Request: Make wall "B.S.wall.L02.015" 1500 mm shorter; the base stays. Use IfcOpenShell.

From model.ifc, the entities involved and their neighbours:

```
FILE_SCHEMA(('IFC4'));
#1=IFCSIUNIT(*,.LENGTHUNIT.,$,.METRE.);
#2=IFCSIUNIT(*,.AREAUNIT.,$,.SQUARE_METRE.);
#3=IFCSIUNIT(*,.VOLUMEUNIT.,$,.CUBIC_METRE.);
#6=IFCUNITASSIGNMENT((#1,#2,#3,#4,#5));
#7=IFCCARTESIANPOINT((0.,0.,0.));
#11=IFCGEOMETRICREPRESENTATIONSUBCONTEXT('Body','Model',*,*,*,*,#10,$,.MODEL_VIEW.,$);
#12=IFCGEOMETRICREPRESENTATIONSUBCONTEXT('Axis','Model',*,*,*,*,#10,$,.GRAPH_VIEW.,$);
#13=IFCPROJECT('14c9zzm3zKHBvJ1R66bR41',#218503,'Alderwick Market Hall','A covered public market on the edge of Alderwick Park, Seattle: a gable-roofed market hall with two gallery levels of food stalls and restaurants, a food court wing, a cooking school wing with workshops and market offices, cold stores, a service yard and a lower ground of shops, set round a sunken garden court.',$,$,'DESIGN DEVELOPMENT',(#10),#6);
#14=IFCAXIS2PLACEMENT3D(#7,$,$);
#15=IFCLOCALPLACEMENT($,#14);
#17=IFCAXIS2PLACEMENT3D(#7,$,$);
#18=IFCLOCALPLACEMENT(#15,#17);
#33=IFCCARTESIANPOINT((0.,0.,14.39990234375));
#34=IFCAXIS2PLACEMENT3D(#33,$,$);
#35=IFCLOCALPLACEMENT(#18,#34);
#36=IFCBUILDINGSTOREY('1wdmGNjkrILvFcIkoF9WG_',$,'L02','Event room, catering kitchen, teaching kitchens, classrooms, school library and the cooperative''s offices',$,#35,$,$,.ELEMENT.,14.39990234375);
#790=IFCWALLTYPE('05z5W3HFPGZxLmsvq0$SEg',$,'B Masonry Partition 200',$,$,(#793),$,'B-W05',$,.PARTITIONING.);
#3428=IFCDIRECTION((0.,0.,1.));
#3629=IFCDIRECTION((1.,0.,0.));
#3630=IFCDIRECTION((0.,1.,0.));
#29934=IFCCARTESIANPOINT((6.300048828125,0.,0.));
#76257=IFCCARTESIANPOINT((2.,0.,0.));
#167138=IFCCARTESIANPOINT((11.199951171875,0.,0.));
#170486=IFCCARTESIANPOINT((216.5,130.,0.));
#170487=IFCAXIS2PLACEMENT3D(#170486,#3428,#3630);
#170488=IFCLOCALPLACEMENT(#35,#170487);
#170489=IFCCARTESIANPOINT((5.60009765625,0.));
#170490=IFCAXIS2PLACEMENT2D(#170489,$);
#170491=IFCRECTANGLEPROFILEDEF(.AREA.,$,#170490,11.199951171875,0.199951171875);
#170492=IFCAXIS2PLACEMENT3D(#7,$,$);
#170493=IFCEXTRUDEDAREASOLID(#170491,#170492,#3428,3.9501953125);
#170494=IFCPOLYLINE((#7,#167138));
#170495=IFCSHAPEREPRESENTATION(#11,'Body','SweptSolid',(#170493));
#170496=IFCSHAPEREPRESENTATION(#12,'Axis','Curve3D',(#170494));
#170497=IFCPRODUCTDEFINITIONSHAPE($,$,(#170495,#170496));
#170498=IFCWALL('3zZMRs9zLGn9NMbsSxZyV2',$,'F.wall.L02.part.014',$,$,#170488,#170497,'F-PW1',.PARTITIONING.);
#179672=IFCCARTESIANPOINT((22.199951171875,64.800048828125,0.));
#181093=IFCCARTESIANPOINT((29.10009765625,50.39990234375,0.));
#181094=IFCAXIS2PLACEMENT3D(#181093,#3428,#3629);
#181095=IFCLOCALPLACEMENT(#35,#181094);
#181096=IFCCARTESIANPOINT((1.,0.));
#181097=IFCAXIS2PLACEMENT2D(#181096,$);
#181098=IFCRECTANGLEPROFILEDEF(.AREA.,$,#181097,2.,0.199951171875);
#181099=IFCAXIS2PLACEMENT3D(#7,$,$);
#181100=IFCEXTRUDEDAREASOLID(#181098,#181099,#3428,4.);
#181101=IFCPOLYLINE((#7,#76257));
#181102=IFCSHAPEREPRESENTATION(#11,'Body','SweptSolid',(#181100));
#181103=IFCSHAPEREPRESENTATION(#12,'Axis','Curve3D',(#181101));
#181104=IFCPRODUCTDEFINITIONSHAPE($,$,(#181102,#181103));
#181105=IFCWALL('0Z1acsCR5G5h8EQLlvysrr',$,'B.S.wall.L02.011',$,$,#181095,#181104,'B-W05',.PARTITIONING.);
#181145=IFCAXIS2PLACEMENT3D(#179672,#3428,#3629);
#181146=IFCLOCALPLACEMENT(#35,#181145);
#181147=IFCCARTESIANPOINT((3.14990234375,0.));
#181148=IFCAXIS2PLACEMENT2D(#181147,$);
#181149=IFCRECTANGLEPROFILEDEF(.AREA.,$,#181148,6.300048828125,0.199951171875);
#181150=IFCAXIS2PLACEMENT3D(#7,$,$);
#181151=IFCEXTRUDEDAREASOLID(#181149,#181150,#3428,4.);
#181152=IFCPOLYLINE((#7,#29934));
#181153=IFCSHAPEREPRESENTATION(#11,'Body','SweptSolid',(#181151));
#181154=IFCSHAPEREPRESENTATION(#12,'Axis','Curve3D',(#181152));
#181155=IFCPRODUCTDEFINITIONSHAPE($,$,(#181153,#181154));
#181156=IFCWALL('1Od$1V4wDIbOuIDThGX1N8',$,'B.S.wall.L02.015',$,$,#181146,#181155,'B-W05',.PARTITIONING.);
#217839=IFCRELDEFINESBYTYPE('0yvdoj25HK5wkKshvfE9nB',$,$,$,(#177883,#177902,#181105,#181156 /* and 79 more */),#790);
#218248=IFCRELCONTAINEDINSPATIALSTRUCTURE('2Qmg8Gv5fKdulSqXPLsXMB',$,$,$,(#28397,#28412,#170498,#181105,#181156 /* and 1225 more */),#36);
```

```python
import ifcopenshell
import ifcopenshell.geom
import ifcopenshell.util.representation
import ifcopenshell.util.shape
import ifcopenshell.util.unit

model = ifcopenshell.open("model.ifc")
unit_scale = ifcopenshell.util.unit.calculate_unit_scale(model)
settings = ifcopenshell.geom.settings()


def volume(element):
    """Net volume in cubic metres, openings subtracted."""
    shape = ifcopenshell.geom.create_shape(settings, element)
    return ifcopenshell.util.shape.get_volume(shape.geometry)


wall = model.by_guid("1Od$1V4wDIbOuIDThGX1N8")
before = volume(wall)

body = ifcopenshell.util.representation.get_representation(wall, "Model", "Body")
solid = body.Items[0]
old_height = solid.Depth
solid.Depth -= 1.5 / unit_scale
after = volume(wall)

print(f"height {old_height:g} -> {solid.Depth:g}, volume {before:.3f} -> {after:.3f} m3")

model.write("model_updated.ifc")
```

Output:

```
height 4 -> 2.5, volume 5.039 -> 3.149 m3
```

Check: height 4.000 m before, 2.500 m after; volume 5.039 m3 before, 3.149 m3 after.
